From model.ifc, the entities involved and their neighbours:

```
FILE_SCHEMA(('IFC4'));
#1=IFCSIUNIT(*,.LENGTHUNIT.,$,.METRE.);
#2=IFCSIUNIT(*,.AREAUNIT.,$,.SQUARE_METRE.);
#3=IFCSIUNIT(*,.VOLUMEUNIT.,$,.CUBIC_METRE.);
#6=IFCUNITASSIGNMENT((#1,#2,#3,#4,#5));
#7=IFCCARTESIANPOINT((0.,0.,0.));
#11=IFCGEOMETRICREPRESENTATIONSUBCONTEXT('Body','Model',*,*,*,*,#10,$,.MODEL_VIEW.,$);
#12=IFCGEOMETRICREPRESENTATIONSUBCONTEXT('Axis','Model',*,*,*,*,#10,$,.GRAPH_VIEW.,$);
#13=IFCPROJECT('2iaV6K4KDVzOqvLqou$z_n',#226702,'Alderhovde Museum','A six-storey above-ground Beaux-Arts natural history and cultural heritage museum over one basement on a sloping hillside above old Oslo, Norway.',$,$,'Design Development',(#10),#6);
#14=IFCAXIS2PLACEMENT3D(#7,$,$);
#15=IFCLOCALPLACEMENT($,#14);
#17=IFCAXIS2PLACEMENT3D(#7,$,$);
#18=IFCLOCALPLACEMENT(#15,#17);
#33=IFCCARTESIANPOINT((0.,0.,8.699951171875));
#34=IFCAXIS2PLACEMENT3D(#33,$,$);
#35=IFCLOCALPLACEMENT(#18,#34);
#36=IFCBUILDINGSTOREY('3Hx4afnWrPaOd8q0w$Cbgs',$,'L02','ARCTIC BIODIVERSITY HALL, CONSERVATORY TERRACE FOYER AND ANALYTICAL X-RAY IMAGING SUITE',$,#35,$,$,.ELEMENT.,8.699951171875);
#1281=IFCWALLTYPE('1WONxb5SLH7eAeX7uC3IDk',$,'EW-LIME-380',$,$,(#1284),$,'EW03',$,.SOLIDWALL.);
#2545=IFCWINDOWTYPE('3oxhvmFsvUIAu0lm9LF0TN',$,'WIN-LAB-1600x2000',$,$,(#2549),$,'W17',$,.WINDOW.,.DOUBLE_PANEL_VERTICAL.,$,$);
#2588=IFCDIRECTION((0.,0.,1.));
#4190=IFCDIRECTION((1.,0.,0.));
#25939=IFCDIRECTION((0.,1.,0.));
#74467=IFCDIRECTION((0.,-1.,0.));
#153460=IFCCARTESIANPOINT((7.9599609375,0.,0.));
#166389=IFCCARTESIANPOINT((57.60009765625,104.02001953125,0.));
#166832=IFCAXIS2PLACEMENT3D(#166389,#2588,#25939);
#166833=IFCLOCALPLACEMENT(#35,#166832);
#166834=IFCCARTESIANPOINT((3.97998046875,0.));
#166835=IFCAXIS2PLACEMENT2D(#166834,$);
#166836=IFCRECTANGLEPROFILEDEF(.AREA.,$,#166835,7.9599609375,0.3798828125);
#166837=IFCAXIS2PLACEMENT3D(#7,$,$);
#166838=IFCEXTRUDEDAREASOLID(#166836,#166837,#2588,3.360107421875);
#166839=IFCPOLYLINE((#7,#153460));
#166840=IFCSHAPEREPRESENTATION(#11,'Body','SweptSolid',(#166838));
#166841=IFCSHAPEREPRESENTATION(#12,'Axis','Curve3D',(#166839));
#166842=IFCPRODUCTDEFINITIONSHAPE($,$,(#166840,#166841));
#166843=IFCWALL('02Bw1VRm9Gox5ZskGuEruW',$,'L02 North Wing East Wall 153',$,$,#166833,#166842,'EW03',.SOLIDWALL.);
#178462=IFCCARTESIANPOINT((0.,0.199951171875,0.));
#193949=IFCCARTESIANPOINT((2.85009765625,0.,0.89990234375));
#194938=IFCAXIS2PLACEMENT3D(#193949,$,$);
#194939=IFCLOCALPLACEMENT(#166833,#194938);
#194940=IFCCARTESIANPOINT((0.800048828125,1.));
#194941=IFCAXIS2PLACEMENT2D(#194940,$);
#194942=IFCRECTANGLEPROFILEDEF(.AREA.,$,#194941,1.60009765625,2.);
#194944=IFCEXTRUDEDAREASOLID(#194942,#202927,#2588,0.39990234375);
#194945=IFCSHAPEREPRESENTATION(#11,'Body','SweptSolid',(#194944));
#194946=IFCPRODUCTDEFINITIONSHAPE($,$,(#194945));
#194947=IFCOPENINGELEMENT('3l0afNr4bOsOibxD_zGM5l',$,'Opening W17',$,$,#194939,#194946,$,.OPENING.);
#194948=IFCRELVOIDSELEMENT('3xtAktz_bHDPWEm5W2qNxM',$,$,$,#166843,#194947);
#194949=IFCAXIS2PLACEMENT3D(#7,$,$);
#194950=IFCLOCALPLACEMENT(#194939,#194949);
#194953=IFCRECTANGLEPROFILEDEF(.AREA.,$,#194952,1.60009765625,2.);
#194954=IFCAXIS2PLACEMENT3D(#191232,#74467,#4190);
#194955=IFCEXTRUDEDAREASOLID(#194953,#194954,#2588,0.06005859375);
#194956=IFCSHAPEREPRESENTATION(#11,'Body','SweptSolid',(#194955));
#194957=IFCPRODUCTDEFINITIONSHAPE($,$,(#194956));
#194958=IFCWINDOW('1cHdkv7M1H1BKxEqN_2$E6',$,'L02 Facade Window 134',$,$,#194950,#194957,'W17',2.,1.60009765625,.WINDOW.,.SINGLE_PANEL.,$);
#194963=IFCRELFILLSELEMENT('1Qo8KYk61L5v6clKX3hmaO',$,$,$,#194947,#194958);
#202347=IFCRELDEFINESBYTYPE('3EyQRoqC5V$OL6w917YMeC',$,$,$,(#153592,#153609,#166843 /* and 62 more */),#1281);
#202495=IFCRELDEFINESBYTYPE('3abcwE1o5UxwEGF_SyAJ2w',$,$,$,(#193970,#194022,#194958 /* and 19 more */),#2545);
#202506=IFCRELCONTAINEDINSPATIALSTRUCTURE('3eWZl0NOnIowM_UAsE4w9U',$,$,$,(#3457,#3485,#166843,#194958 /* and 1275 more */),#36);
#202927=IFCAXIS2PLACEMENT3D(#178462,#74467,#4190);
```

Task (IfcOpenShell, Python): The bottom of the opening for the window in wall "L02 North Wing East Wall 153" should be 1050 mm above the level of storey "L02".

```python
import numpy as np
import ifcopenshell
import ifcopenshell.api.geometry
import ifcopenshell.geom
import ifcopenshell.util.element
import ifcopenshell.util.placement
import ifcopenshell.util.shape
import ifcopenshell.util.unit

model = ifcopenshell.open("model.ifc")
unit_scale = ifcopenshell.util.unit.calculate_unit_scale(model)

window = model.by_guid("1cHdkv7M1H1BKxEqN_2$E6")
opening = window.FillsVoids[0].RelatingOpeningElement
storey = ifcopenshell.util.element.get_container(window, ifc_class="IfcBuildingStorey")
level = ifcopenshell.util.placement.get_local_placement(storey.ObjectPlacement)[2, 3]

# The opening's origin need not be at the sill, so measure its lowest point.
shape = ifcopenshell.geom.create_shape(ifcopenshell.geom.settings(), opening)
bottom = ifcopenshell.util.shape.get_shape_bottom_elevation(shape, shape.geometry) / unit_scale
dz = level + 1.05 / unit_scale - bottom

shift = np.array([0.0, 0.0, dz])
# The window is placed relative to its opening, so it follows when the opening moves.
matrix = ifcopenshell.util.placement.get_local_placement(opening.ObjectPlacement)
matrix[:3, 3] += shift
ifcopenshell.api.geometry.edit_object_placement(
    model, product=opening, matrix=matrix, is_si=False, should_transform_children=True
)

print(f"moved by {dz * unit_scale:+.3f} m")

model.write("model_updated.ifc")
```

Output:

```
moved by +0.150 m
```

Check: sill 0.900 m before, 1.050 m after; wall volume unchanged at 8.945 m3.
